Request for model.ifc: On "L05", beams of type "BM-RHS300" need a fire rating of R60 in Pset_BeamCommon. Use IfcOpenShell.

First a look at what the model holds.

```python
import ifcopenshell
import ifcopenshell.util.element

model = ifcopenshell.open("model.ifc")
print(model.schema)
storey = next(s for s in model.by_type("IfcBuildingStorey") if s.Name == "L05")
beams = [e for e in ifcopenshell.util.element.get_decomposition(storey) if e.is_a("IfcBeam")]
seen = {}
for e in beams:
    element_type = ifcopenshell.util.element.get_type(e)
    key = (element_type.Name if element_type != e and element_type else None, ifcopenshell.util.element.get_pset(e, "Pset_BeamCommon", "FireRating"))
    seen[key] = seen.get(key, 0) + 1
for (name, value), count in sorted(seen.items(), key=str):
    print(count, "x", name, "|", value)
```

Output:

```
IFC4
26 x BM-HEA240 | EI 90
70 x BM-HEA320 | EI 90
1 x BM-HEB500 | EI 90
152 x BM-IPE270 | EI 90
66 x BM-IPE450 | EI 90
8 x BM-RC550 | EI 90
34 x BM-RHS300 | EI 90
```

```python
import ifcopenshell
import ifcopenshell.api.pset
import ifcopenshell.util.element

model = ifcopenshell.open("model.ifc")

storey = next(s for s in model.by_type("IfcBuildingStorey") if s.Name == "L05")
beams = [e for e in ifcopenshell.util.element.get_decomposition(storey) if e.is_a("IfcBeam")]

count = 0
for e in beams:
    element_type = ifcopenshell.util.element.get_type(e)
    if element_type in (None, e) or element_type.Name != "BM-RHS300":
        continue
    # add_pset returns the element's existing set when there is one.
    pset = ifcopenshell.api.pset.add_pset(model, product=e, name="Pset_BeamCommon")
    ifcopenshell.api.pset.edit_pset(model, pset=pset, properties={"FireRating": "R60"})
    count += 1

print(count, "beams updated")

model.write("model_rev.ifc")
```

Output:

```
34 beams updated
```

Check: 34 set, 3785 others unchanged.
